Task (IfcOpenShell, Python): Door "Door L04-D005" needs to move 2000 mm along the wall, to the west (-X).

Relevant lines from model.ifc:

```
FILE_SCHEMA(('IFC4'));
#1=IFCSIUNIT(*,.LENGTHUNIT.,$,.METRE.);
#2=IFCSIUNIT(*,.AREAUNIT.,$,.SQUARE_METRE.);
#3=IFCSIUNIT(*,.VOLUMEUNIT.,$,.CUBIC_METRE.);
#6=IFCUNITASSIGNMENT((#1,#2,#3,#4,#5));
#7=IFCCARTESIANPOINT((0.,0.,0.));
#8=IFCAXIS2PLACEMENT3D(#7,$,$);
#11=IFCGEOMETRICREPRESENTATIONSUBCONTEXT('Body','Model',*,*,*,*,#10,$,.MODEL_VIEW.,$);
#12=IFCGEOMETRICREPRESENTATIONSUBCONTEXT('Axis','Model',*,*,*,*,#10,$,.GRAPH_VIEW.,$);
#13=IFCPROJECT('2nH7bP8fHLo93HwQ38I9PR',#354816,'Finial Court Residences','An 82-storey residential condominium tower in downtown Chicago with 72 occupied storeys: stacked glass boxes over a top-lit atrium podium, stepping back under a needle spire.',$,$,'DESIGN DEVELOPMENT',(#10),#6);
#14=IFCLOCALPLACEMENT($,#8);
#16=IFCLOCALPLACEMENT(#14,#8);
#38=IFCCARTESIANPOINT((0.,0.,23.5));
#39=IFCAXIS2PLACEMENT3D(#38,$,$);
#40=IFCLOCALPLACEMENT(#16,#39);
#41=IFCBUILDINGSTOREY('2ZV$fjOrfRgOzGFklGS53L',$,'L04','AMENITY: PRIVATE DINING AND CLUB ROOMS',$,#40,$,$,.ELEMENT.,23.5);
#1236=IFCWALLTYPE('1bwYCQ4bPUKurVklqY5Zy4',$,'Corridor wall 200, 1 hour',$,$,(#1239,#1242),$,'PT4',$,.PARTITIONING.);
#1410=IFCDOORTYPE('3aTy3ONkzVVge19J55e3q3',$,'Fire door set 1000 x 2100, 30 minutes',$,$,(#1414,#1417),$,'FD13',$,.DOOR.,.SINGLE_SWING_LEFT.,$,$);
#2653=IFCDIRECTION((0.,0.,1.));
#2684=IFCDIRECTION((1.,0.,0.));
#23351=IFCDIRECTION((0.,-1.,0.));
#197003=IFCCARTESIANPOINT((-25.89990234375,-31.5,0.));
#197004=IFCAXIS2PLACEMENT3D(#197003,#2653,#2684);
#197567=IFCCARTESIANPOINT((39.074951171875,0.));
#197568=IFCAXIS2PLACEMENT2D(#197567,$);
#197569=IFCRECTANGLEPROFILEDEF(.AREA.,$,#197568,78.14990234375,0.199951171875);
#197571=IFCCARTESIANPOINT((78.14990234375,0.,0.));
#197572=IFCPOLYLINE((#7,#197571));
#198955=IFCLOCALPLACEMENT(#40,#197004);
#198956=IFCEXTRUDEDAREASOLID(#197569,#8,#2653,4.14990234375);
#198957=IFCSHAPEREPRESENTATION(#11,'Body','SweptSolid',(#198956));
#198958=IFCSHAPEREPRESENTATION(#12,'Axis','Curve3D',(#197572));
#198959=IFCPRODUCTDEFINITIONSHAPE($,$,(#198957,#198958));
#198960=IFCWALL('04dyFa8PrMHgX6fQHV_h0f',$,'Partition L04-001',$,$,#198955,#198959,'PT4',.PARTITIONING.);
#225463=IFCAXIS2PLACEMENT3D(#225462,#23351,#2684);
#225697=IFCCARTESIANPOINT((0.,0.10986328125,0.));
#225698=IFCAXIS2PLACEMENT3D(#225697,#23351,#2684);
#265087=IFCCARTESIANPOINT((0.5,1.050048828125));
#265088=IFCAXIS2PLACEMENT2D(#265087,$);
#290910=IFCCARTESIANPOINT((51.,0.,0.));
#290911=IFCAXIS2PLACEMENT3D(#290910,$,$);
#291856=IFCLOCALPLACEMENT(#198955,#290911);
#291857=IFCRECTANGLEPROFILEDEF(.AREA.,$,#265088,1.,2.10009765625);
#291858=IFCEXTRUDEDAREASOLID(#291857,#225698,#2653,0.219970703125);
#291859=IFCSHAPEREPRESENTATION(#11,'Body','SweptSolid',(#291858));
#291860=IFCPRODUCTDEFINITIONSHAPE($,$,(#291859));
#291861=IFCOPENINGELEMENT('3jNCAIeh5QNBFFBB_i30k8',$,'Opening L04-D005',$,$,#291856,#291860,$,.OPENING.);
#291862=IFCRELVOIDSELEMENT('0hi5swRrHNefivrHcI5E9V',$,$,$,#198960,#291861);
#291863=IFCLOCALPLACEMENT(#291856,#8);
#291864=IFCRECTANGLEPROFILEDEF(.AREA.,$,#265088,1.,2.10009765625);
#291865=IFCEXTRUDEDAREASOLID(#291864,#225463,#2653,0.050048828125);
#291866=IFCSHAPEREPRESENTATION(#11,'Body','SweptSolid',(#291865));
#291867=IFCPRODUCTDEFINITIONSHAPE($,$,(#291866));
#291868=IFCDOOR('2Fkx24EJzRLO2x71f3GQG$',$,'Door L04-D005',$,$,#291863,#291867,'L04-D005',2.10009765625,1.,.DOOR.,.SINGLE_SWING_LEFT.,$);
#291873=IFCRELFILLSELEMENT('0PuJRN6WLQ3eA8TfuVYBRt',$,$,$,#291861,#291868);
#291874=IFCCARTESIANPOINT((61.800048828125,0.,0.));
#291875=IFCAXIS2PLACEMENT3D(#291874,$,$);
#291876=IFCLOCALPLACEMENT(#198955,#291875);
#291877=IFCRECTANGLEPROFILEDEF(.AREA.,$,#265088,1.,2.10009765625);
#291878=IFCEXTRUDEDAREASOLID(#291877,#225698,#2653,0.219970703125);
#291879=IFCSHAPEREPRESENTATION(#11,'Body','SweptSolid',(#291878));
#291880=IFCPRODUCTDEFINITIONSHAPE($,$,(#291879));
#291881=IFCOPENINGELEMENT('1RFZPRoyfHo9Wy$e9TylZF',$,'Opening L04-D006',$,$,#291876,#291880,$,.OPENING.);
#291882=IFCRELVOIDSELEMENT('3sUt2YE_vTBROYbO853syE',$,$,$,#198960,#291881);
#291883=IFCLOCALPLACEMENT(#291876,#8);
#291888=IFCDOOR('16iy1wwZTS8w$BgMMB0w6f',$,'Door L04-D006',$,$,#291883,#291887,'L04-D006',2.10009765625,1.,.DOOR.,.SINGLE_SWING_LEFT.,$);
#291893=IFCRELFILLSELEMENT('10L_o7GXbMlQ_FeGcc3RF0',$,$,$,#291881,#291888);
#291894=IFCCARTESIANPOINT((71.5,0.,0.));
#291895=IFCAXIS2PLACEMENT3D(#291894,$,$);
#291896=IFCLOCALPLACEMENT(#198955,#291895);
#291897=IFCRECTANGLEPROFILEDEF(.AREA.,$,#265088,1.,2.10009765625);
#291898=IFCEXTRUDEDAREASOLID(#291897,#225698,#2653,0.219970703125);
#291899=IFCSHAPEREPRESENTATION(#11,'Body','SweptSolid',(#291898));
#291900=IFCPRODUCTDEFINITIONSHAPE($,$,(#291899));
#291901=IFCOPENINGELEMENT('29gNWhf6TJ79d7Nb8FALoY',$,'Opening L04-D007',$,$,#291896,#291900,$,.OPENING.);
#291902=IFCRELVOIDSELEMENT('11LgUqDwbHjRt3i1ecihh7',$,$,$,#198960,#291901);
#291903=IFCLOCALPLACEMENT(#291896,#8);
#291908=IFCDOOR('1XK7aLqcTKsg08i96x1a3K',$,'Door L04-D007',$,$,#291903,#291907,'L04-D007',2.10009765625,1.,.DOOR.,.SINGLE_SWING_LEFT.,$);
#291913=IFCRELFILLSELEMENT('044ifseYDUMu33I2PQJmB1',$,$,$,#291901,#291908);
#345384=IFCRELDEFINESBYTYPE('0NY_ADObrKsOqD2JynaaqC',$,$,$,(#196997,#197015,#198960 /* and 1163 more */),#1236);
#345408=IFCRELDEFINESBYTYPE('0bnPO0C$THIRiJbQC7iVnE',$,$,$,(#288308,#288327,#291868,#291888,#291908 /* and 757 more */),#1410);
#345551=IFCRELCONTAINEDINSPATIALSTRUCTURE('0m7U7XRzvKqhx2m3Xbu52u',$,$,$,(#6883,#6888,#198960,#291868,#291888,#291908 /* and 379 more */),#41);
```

```python
import ifcopenshell
import ifcopenshell.api.geometry
import ifcopenshell.util.placement
import ifcopenshell.util.unit

model = ifcopenshell.open("model.ifc")
unit_scale = ifcopenshell.util.unit.calculate_unit_scale(model)

door = model.by_guid("2Fkx24EJzRLO2x71f3GQG$")
opening = door.FillsVoids[0].RelatingOpeningElement
wall = opening.VoidsElements[0].RelatingBuildingElement

wall_matrix = ifcopenshell.util.placement.get_local_placement(wall.ObjectPlacement)
shift = wall_matrix[:3, 0] * -2 / unit_scale
before = ifcopenshell.util.placement.get_local_placement(door.ObjectPlacement)[:3, 3].copy()

# The door is placed relative to its opening, so it follows when the opening moves.
matrix = ifcopenshell.util.placement.get_local_placement(opening.ObjectPlacement)
matrix[:3, 3] += shift
ifcopenshell.api.geometry.edit_object_placement(
    model, product=opening, matrix=matrix, is_si=False, should_transform_children=True
)

after = ifcopenshell.util.placement.get_local_placement(door.ObjectPlacement)[:3, 3]
print("door moved by", (after - before).round(3) + 0.0)

model.write("model-out.ifc")
```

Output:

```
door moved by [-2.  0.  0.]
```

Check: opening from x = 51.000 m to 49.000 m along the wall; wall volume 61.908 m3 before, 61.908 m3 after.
